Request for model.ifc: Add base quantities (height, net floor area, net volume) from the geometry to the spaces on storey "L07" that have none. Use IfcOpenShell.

First a look at what the model holds.

```python
import ifcopenshell
import ifcopenshell.util.element
import ifcopenshell.util.unit

model = ifcopenshell.open("model.ifc")
print(model.schema)
for unit_type in ("LENGTHUNIT", "AREAUNIT", "VOLUMEUNIT"):
    print(unit_type, ifcopenshell.util.unit.calculate_unit_scale(model, unit_type))
storey = next(s for s in model.by_type("IfcBuildingStorey") if s.Name == "L07")
spaces = [e for e in ifcopenshell.util.element.get_decomposition(storey) if e.is_a("IfcSpace")]
for e in sorted(spaces, key=lambda e: e.id()):
    print(e.id(), e.is_a(), e.Name, list(ifcopenshell.util.element.get_psets(e, qtos_only=True)), sep=" | ")
```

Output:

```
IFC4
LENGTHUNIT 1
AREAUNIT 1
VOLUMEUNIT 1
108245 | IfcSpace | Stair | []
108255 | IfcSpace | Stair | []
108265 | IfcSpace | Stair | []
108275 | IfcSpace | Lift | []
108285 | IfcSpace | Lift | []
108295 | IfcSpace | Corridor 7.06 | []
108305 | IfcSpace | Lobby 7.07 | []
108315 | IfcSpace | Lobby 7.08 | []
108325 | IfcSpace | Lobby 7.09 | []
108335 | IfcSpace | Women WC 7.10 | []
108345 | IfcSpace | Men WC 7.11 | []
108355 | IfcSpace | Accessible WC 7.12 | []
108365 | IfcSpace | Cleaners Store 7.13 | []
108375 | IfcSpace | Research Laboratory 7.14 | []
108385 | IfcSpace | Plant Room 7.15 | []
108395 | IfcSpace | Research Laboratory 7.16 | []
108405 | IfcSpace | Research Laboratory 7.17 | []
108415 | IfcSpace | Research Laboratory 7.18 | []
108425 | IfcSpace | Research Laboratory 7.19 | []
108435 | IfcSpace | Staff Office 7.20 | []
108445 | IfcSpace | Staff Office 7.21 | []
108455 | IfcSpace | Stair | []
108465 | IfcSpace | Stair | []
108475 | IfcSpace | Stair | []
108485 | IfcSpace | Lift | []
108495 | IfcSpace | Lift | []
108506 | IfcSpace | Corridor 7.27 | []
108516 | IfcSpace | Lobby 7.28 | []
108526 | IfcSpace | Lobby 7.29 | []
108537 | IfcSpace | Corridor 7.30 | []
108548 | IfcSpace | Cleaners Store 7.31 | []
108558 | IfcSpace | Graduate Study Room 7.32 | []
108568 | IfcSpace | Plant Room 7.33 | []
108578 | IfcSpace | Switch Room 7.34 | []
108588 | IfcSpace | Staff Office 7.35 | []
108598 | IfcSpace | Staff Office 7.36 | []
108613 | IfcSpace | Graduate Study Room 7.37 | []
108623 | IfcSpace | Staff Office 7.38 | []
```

```python
import ifcopenshell
import ifcopenshell.api.pset
import ifcopenshell.geom
import ifcopenshell.util.element
import ifcopenshell.util.shape
import ifcopenshell.util.unit

model = ifcopenshell.open("model.ifc")
unit_scale = ifcopenshell.util.unit.calculate_unit_scale(model)
area_scale = ifcopenshell.util.unit.calculate_unit_scale(model, "AREAUNIT")
volume_scale = ifcopenshell.util.unit.calculate_unit_scale(model, "VOLUMEUNIT")
settings = ifcopenshell.geom.settings()

storey = next(s for s in model.by_type("IfcBuildingStorey") if s.Name == "L07")
spaces = [e for e in ifcopenshell.util.element.get_decomposition(storey) if e.is_a("IfcSpace")]

for e in sorted(spaces, key=lambda e: e.id()):
    if ifcopenshell.util.element.get_psets(e, qtos_only=True, should_inherit=False):
        continue
    # Geometry comes back in metres, in the element's own axes.
    shape = ifcopenshell.geom.create_shape(settings, e)
    values = {
        "Height": ifcopenshell.util.shape.get_z(shape.geometry) / unit_scale,
        "NetFloorArea": ifcopenshell.util.shape.get_footprint_area(shape.geometry) / area_scale,
        "NetVolume": ifcopenshell.util.shape.get_volume(shape.geometry) / volume_scale,
    }
    qto = ifcopenshell.api.pset.add_qto(model, product=e, name="Qto_SpaceBaseQuantities")
    ifcopenshell.api.pset.edit_qto(model, qto=qto, properties=values)
    print(e.id(), {k: round(v, 3) for k, v in values.items()})

model.write("model_edited.ifc")
```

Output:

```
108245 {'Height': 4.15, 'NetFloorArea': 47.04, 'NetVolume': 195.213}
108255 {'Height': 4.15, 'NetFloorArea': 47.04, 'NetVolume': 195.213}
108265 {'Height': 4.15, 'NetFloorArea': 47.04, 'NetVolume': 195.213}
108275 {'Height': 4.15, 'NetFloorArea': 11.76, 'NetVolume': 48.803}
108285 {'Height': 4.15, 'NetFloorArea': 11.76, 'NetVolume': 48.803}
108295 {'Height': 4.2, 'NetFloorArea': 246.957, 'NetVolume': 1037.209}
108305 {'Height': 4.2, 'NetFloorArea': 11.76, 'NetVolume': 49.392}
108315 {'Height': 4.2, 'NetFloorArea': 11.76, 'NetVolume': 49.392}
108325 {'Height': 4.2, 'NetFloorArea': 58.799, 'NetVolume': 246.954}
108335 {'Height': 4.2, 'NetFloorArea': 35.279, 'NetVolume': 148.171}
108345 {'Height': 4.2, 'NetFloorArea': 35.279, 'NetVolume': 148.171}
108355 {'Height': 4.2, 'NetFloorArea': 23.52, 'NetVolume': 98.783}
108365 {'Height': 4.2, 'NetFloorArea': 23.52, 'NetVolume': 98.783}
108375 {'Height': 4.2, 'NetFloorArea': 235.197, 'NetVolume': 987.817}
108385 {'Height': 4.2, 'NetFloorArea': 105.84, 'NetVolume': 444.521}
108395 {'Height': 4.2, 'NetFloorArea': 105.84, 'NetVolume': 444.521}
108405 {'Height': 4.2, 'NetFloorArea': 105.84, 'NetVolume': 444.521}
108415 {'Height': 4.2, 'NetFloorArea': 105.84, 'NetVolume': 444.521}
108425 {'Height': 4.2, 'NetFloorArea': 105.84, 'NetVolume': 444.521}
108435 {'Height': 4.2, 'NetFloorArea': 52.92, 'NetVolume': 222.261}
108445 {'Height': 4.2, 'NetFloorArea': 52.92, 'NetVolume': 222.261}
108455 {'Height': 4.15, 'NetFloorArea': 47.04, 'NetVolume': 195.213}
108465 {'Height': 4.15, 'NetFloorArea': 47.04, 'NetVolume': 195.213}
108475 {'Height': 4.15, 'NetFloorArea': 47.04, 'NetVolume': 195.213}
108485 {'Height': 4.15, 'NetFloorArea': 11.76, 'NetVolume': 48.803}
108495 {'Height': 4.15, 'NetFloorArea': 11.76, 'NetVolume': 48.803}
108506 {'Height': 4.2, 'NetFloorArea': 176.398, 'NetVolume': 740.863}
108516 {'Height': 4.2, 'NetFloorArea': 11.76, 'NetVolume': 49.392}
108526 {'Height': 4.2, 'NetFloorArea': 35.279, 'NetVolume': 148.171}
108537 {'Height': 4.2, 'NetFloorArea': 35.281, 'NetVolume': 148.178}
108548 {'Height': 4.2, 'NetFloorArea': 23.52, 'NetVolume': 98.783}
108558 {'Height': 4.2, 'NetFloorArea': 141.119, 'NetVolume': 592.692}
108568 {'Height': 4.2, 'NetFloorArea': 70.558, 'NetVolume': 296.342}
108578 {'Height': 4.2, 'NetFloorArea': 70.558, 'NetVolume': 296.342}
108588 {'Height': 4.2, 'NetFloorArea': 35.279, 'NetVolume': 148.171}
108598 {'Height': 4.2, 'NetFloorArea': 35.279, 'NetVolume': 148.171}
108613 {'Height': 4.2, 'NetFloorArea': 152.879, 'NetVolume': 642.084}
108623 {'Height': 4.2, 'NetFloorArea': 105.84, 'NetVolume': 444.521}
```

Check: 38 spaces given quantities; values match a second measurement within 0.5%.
